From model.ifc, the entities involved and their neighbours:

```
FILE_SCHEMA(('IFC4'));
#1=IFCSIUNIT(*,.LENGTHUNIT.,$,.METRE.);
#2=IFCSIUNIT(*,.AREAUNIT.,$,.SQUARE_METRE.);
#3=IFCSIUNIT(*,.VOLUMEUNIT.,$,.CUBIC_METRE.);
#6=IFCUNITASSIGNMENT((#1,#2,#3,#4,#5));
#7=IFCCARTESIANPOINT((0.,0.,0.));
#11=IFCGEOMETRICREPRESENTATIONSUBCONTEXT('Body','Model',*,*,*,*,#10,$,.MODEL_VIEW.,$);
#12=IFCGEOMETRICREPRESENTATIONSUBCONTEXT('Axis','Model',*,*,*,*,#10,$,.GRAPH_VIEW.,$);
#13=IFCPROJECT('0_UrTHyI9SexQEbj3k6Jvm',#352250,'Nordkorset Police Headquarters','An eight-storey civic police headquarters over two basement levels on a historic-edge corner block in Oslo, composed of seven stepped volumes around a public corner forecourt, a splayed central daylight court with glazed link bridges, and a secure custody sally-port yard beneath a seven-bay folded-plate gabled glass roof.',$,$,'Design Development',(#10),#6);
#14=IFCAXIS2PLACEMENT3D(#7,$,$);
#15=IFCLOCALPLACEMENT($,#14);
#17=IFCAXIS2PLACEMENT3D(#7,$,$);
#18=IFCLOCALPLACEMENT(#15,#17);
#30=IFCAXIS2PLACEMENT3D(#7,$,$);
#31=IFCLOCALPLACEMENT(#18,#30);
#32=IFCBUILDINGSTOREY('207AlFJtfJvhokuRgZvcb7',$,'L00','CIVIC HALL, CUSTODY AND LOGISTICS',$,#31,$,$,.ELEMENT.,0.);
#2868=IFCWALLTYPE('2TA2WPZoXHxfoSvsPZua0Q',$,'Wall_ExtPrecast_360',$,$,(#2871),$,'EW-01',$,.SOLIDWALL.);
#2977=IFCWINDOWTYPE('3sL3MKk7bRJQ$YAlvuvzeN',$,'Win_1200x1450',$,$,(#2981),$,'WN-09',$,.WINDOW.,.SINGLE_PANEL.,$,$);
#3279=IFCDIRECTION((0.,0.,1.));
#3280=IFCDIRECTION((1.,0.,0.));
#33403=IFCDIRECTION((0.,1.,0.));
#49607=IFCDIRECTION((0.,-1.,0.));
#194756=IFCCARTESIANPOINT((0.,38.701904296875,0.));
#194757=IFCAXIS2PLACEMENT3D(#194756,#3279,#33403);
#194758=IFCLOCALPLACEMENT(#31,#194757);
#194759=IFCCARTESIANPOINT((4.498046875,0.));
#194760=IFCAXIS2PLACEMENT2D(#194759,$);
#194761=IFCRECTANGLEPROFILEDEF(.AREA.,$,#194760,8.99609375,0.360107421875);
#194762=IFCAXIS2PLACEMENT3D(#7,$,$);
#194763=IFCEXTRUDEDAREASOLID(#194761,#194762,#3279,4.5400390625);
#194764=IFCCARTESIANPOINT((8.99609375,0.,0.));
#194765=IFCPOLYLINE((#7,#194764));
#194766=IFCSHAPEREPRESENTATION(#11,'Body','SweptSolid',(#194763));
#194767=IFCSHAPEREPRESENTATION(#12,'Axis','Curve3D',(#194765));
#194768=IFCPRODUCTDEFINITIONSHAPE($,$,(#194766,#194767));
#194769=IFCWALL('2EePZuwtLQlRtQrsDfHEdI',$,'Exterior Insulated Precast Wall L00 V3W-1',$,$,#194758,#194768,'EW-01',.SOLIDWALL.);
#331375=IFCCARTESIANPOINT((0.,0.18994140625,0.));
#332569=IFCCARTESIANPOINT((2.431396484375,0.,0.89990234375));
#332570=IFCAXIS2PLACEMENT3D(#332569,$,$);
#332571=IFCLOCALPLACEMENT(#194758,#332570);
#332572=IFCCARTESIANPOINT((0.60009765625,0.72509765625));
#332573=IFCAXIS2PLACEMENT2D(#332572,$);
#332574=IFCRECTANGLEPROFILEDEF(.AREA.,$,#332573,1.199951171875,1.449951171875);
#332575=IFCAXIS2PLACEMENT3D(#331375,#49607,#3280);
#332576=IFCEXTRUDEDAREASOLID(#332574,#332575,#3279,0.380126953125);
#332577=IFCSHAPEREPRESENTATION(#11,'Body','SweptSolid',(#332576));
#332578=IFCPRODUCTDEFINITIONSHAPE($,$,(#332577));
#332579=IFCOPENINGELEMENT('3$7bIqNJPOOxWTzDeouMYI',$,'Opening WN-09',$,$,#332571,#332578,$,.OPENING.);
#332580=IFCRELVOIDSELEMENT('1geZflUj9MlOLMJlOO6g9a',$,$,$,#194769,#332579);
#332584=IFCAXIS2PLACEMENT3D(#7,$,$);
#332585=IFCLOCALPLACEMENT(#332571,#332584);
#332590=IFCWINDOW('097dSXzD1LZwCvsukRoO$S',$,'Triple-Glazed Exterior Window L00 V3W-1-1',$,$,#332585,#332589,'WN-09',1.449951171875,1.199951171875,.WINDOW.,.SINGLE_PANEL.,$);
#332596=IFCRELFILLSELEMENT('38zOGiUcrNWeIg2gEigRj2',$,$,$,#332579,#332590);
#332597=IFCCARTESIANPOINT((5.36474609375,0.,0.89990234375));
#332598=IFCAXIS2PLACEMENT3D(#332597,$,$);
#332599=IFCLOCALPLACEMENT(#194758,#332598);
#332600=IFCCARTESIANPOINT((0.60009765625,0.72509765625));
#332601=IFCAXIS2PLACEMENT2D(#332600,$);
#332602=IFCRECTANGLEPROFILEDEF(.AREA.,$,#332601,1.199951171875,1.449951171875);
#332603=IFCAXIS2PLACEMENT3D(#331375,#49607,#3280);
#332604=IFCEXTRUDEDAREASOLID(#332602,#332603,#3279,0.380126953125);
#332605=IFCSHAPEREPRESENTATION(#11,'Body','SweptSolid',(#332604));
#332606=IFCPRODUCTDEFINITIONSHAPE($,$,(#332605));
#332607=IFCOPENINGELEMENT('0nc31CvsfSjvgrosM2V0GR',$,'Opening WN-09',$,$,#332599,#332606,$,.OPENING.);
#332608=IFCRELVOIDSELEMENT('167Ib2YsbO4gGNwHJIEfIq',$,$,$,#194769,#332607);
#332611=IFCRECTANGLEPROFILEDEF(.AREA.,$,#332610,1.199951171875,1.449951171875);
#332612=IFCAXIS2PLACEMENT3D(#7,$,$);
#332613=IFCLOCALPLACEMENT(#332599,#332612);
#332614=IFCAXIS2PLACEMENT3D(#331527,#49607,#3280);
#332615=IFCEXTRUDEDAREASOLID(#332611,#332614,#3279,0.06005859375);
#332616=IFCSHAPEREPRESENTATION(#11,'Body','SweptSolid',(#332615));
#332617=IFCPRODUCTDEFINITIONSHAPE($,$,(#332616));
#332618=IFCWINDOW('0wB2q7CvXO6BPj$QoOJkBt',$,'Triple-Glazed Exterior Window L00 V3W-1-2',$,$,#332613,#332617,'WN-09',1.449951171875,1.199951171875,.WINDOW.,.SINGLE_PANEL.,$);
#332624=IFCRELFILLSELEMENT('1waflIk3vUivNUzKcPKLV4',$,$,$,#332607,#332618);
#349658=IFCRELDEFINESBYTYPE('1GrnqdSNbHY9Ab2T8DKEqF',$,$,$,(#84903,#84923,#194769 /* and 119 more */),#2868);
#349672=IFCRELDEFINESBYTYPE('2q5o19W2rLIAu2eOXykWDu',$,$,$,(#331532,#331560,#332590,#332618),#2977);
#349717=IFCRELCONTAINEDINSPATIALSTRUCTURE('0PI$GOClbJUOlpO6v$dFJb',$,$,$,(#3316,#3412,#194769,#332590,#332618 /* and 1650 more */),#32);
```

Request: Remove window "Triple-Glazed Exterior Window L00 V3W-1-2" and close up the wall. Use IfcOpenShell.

```python
import ifcopenshell
import ifcopenshell.api.feature
import ifcopenshell.api.root
import ifcopenshell.geom
import ifcopenshell.util.shape

model = ifcopenshell.open("model.ifc")
settings = ifcopenshell.geom.settings()


def volume(element):
    """Net volume in cubic metres, openings subtracted."""
    shape = ifcopenshell.geom.create_shape(settings, element)
    return ifcopenshell.util.shape.get_volume(shape.geometry)


window = model.by_id(332618)
opening = window.FillsVoids[0].RelatingOpeningElement
wall = opening.VoidsElements[0].RelatingBuildingElement
before = volume(wall)

ifcopenshell.api.root.remove_product(model, product=window)
ifcopenshell.api.feature.remove_feature(model, feature=opening)

after = volume(wall)

print(f"wall volume {before:.3f} -> {after:.3f} m3")

model.write("model_v2.ifc")
```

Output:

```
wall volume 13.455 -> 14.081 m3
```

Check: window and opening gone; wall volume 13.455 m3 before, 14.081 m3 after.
